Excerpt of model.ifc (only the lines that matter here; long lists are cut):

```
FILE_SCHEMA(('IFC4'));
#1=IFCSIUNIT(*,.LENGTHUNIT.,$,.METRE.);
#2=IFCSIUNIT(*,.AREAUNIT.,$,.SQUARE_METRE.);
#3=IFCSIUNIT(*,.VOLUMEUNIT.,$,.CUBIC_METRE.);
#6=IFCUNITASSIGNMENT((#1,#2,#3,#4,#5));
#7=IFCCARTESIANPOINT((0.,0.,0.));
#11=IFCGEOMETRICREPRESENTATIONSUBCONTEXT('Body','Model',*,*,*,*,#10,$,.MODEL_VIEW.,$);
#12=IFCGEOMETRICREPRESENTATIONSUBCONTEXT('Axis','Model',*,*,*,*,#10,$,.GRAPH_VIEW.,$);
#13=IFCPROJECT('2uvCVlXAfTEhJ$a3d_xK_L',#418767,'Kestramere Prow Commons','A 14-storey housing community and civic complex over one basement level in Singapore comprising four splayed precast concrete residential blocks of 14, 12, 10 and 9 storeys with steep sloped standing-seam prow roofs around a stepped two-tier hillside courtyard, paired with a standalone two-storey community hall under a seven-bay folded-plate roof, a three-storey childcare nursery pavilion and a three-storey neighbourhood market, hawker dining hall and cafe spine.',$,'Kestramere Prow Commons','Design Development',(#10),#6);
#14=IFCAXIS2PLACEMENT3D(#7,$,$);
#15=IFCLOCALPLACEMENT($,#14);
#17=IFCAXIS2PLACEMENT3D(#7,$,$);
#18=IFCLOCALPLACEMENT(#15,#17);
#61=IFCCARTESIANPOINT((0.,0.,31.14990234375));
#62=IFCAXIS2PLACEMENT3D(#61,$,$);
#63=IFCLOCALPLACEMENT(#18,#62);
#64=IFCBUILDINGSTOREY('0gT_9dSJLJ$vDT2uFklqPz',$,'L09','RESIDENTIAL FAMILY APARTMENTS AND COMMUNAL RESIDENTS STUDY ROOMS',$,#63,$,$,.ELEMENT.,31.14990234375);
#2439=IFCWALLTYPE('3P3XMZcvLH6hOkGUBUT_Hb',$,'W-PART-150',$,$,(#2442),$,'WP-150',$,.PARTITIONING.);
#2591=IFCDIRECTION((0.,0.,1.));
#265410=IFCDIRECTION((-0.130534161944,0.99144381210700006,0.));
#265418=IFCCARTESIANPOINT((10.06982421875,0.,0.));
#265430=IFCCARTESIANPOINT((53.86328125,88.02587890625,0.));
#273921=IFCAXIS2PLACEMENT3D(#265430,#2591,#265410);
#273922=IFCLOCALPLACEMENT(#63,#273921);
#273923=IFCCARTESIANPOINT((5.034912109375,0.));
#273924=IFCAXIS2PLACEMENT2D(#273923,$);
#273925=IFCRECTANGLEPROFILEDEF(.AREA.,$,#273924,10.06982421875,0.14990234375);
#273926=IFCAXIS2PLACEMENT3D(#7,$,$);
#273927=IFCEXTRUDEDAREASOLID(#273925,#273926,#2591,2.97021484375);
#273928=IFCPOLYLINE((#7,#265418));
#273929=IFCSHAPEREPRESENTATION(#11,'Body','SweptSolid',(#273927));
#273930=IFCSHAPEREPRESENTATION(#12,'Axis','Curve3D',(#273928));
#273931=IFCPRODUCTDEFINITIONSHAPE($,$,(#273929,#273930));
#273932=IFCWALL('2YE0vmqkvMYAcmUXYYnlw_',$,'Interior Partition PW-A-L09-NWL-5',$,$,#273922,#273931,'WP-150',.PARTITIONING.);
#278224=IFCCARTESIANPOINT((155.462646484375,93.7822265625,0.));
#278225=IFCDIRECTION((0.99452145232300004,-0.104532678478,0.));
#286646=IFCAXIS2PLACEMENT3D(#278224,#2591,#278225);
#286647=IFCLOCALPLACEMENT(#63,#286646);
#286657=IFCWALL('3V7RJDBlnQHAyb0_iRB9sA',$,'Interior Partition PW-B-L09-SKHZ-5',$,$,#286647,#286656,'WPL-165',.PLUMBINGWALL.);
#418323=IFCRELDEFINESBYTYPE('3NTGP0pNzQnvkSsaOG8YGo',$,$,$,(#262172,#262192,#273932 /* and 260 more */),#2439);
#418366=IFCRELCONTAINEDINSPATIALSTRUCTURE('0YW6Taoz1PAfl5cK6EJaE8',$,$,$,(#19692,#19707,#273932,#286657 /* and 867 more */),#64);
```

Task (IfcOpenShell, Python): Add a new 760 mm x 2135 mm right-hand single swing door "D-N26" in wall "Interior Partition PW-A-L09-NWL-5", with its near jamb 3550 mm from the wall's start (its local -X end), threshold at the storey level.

```python
import numpy as np
import ifcopenshell
import ifcopenshell.api.feature
import ifcopenshell.api.geometry
import ifcopenshell.api.root
import ifcopenshell.api.spatial
import ifcopenshell.geom
import ifcopenshell.util.element
import ifcopenshell.util.placement
import ifcopenshell.util.representation
import ifcopenshell.util.shape
import ifcopenshell.util.unit

model = ifcopenshell.open("model.ifc")
unit_scale = ifcopenshell.util.unit.calculate_unit_scale(model)
settings = ifcopenshell.geom.settings()


def volume(element):
    """Net volume in cubic metres, openings subtracted."""
    shape = ifcopenshell.geom.create_shape(settings, element)
    return ifcopenshell.util.shape.get_volume(shape.geometry)


wall = model.by_guid("2YE0vmqkvMYAcmUXYYnlw_")
storey = ifcopenshell.util.element.get_container(wall, ifc_class="IfcBuildingStorey")
context = ifcopenshell.util.representation.get_context(model, "Model", "Body", "MODEL_VIEW")
before = volume(wall)

width, height, from_end, sill = 0.76, 2.135, 3.55, 0.0  # metres

# The wall runs along its own X axis, and the end named is its -X end.
wall_shape = ifcopenshell.geom.create_shape(settings, wall)
x, y, z = ifcopenshell.util.shape.get_vertices(wall_shape.geometry).T
start = x.min() + from_end
face, thickness = float(y.min()), float(y.max() - y.min())
wall_matrix = ifcopenshell.util.placement.get_local_placement(wall.ObjectPlacement)
level = ifcopenshell.util.placement.get_local_placement(storey.ObjectPlacement)[2, 3]


def in_wall(x, y):
    """Placement at x, y metres in the wall's axes, at sill height."""
    matrix = wall_matrix.copy()
    matrix[:, 3] = wall_matrix @ np.array([x / unit_scale, y / unit_scale, 0.0, 1.0])
    matrix[2, 3] = level + sill / unit_scale
    return matrix


# Opening: a box that overshoots both wall faces by 50 mm.
opening = ifcopenshell.api.root.create_entity(model, ifc_class="IfcOpeningElement", predefined_type="OPENING")
box = ifcopenshell.api.geometry.add_wall_representation(
    model, context=context, length=width, height=height, thickness=thickness + 0.1
)
ifcopenshell.api.geometry.assign_representation(model, product=opening, representation=box)
ifcopenshell.api.geometry.edit_object_placement(model, product=opening, matrix=in_wall(start, face - 0.05), is_si=False)
ifcopenshell.api.feature.add_feature(model, feature=opening, element=wall)

door = ifcopenshell.api.root.create_entity(model, ifc_class="IfcDoor", name="D-N26", predefined_type="DOOR")
door.OverallWidth, door.OverallHeight = width / unit_scale, height / unit_scale
door.OperationType = "SINGLE_SWING_RIGHT"
body = ifcopenshell.api.geometry.add_door_representation(
    model,
    context=context,
    overall_width=door.OverallWidth,
    overall_height=door.OverallHeight,
    operation_type="SINGLE_SWING_RIGHT",
    lining_properties={"LiningDepth": thickness / unit_scale, "ThresholdDepth": thickness / unit_scale},
)
ifcopenshell.api.geometry.assign_representation(model, product=door, representation=body)
ifcopenshell.api.spatial.assign_container(model, products=[door], relating_structure=storey)
ifcopenshell.api.feature.add_filling(model, opening=opening, element=door)

# The lining spans the wall, so the door starts at the wall face.
ifcopenshell.api.geometry.edit_object_placement(model, product=door, matrix=in_wall(start, face), is_si=False)

after = volume(wall)

print(f"wall volume {before:.3f} -> {after:.3f} m3")

model.write("model_v2.ifc")
```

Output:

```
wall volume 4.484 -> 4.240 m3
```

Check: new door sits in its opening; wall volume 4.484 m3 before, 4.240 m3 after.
